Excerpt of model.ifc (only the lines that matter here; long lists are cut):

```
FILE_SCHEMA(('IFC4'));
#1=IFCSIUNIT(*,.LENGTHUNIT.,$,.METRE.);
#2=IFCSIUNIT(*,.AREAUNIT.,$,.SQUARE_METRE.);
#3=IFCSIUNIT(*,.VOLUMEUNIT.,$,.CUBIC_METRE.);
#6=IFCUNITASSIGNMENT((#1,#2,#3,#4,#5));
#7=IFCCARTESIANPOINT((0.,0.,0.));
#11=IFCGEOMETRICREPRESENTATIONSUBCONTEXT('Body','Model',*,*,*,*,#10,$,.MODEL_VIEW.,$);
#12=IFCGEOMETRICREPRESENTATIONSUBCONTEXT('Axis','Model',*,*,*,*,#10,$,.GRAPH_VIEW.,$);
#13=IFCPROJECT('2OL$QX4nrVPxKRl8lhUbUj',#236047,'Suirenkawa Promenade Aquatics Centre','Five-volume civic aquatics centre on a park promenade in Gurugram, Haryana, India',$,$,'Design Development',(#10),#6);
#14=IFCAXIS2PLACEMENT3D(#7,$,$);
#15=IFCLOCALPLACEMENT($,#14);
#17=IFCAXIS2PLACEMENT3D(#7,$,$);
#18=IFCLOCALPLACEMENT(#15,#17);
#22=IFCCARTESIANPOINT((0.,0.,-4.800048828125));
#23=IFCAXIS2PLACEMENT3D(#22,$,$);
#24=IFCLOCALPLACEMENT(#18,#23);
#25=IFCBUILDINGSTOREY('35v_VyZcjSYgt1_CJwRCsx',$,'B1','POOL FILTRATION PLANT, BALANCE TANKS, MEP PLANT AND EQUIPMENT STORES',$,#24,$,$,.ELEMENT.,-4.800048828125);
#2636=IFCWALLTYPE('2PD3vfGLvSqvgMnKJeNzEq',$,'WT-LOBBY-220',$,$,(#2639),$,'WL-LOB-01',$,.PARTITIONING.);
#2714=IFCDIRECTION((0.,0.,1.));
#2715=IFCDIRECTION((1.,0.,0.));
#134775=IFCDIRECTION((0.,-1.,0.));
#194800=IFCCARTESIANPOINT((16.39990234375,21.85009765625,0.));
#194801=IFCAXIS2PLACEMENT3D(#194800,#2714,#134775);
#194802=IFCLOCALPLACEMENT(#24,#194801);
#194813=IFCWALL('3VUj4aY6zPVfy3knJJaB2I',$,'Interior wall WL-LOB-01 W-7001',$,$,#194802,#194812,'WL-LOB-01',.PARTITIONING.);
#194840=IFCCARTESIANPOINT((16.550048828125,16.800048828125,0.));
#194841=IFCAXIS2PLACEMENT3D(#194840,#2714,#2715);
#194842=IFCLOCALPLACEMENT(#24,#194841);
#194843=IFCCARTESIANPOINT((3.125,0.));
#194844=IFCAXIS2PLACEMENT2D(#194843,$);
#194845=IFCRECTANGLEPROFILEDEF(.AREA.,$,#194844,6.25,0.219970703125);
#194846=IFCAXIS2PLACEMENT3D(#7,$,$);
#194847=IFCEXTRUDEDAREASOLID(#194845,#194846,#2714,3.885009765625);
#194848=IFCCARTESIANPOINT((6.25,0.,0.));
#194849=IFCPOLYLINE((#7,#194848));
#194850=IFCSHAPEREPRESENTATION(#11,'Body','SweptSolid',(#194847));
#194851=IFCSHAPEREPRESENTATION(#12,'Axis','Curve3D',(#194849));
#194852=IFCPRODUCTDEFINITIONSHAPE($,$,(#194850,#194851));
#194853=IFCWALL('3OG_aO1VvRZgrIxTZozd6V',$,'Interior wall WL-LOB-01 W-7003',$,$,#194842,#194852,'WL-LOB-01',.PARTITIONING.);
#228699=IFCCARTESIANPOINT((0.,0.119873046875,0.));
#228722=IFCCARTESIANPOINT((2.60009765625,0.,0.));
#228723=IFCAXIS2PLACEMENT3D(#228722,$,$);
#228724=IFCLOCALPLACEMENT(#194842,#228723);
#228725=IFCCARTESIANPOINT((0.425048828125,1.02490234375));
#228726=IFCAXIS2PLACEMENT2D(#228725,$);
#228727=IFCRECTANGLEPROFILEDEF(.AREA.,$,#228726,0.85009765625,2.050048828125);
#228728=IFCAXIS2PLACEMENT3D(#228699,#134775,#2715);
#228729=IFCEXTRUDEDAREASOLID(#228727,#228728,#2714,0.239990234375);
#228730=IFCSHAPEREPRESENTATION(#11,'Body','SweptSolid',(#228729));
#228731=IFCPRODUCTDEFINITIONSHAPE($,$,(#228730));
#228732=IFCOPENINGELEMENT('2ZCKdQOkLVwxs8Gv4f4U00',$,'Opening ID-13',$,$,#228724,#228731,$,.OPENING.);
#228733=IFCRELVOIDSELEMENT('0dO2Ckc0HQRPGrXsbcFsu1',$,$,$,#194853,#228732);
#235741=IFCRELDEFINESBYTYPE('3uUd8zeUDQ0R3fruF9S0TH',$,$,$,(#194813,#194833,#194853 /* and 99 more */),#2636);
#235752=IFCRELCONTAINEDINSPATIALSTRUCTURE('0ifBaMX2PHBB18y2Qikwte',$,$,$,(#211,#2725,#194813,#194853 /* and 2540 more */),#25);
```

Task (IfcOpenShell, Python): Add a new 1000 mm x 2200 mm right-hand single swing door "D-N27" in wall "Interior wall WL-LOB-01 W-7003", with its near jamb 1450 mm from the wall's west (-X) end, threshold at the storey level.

```python
import numpy as np
import ifcopenshell
import ifcopenshell.api.feature
import ifcopenshell.api.geometry
import ifcopenshell.api.root
import ifcopenshell.api.spatial
import ifcopenshell.geom
import ifcopenshell.util.element
import ifcopenshell.util.placement
import ifcopenshell.util.representation
import ifcopenshell.util.shape
import ifcopenshell.util.unit

model = ifcopenshell.open("model.ifc")
unit_scale = ifcopenshell.util.unit.calculate_unit_scale(model)
settings = ifcopenshell.geom.settings()


def volume(element):
    """Net volume in cubic metres, openings subtracted."""
    shape = ifcopenshell.geom.create_shape(settings, element)
    return ifcopenshell.util.shape.get_volume(shape.geometry)


wall = model.by_guid("3OG_aO1VvRZgrIxTZozd6V")
storey = ifcopenshell.util.element.get_container(wall, ifc_class="IfcBuildingStorey")
context = ifcopenshell.util.representation.get_context(model, "Model", "Body", "MODEL_VIEW")
before = volume(wall)

width, height, from_end, sill = 1, 2.2, 1.45, 0.0  # metres

# The wall runs along its own X axis, and the end named is its -X end.
wall_shape = ifcopenshell.geom.create_shape(settings, wall)
x, y, z = ifcopenshell.util.shape.get_vertices(wall_shape.geometry).T
start = x.min() + from_end
face, thickness = float(y.min()), float(y.max() - y.min())
wall_matrix = ifcopenshell.util.placement.get_local_placement(wall.ObjectPlacement)
level = ifcopenshell.util.placement.get_local_placement(storey.ObjectPlacement)[2, 3]


def in_wall(x, y):
    """Placement at x, y metres in the wall's axes, at sill height."""
    matrix = wall_matrix.copy()
    matrix[:, 3] = wall_matrix @ np.array([x / unit_scale, y / unit_scale, 0.0, 1.0])
    matrix[2, 3] = level + sill / unit_scale
    return matrix


# Opening: a box that overshoots both wall faces by 50 mm.
opening = ifcopenshell.api.root.create_entity(model, ifc_class="IfcOpeningElement", predefined_type="OPENING")
box = ifcopenshell.api.geometry.add_wall_representation(
    model, context=context, length=width, height=height, thickness=thickness + 0.1
)
ifcopenshell.api.geometry.assign_representation(model, product=opening, representation=box)
ifcopenshell.api.geometry.edit_object_placement(model, product=opening, matrix=in_wall(start, face - 0.05), is_si=False)
ifcopenshell.api.feature.add_feature(model, feature=opening, element=wall)

door = ifcopenshell.api.root.create_entity(model, ifc_class="IfcDoor", name="D-N27", predefined_type="DOOR")
door.OverallWidth, door.OverallHeight = width / unit_scale, height / unit_scale
door.OperationType = "SINGLE_SWING_RIGHT"
body = ifcopenshell.api.geometry.add_door_representation(
    model,
    context=context,
    overall_width=door.OverallWidth,
    overall_height=door.OverallHeight,
    operation_type="SINGLE_SWING_RIGHT",
    lining_properties={"LiningDepth": thickness / unit_scale, "ThresholdDepth": thickness / unit_scale},
)
ifcopenshell.api.geometry.assign_representation(model, product=door, representation=body)
ifcopenshell.api.spatial.assign_container(model, products=[door], relating_structure=storey)
ifcopenshell.api.feature.add_filling(model, opening=opening, element=door)

# The lining spans the wall, so the door starts at the wall face.
ifcopenshell.api.geometry.edit_object_placement(model, product=door, matrix=in_wall(start, face), is_si=False)

after = volume(wall)

print(f"wall volume {before:.3f} -> {after:.3f} m3")

model.write("model-out.ifc")
```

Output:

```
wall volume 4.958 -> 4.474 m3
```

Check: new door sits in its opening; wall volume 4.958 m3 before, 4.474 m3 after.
